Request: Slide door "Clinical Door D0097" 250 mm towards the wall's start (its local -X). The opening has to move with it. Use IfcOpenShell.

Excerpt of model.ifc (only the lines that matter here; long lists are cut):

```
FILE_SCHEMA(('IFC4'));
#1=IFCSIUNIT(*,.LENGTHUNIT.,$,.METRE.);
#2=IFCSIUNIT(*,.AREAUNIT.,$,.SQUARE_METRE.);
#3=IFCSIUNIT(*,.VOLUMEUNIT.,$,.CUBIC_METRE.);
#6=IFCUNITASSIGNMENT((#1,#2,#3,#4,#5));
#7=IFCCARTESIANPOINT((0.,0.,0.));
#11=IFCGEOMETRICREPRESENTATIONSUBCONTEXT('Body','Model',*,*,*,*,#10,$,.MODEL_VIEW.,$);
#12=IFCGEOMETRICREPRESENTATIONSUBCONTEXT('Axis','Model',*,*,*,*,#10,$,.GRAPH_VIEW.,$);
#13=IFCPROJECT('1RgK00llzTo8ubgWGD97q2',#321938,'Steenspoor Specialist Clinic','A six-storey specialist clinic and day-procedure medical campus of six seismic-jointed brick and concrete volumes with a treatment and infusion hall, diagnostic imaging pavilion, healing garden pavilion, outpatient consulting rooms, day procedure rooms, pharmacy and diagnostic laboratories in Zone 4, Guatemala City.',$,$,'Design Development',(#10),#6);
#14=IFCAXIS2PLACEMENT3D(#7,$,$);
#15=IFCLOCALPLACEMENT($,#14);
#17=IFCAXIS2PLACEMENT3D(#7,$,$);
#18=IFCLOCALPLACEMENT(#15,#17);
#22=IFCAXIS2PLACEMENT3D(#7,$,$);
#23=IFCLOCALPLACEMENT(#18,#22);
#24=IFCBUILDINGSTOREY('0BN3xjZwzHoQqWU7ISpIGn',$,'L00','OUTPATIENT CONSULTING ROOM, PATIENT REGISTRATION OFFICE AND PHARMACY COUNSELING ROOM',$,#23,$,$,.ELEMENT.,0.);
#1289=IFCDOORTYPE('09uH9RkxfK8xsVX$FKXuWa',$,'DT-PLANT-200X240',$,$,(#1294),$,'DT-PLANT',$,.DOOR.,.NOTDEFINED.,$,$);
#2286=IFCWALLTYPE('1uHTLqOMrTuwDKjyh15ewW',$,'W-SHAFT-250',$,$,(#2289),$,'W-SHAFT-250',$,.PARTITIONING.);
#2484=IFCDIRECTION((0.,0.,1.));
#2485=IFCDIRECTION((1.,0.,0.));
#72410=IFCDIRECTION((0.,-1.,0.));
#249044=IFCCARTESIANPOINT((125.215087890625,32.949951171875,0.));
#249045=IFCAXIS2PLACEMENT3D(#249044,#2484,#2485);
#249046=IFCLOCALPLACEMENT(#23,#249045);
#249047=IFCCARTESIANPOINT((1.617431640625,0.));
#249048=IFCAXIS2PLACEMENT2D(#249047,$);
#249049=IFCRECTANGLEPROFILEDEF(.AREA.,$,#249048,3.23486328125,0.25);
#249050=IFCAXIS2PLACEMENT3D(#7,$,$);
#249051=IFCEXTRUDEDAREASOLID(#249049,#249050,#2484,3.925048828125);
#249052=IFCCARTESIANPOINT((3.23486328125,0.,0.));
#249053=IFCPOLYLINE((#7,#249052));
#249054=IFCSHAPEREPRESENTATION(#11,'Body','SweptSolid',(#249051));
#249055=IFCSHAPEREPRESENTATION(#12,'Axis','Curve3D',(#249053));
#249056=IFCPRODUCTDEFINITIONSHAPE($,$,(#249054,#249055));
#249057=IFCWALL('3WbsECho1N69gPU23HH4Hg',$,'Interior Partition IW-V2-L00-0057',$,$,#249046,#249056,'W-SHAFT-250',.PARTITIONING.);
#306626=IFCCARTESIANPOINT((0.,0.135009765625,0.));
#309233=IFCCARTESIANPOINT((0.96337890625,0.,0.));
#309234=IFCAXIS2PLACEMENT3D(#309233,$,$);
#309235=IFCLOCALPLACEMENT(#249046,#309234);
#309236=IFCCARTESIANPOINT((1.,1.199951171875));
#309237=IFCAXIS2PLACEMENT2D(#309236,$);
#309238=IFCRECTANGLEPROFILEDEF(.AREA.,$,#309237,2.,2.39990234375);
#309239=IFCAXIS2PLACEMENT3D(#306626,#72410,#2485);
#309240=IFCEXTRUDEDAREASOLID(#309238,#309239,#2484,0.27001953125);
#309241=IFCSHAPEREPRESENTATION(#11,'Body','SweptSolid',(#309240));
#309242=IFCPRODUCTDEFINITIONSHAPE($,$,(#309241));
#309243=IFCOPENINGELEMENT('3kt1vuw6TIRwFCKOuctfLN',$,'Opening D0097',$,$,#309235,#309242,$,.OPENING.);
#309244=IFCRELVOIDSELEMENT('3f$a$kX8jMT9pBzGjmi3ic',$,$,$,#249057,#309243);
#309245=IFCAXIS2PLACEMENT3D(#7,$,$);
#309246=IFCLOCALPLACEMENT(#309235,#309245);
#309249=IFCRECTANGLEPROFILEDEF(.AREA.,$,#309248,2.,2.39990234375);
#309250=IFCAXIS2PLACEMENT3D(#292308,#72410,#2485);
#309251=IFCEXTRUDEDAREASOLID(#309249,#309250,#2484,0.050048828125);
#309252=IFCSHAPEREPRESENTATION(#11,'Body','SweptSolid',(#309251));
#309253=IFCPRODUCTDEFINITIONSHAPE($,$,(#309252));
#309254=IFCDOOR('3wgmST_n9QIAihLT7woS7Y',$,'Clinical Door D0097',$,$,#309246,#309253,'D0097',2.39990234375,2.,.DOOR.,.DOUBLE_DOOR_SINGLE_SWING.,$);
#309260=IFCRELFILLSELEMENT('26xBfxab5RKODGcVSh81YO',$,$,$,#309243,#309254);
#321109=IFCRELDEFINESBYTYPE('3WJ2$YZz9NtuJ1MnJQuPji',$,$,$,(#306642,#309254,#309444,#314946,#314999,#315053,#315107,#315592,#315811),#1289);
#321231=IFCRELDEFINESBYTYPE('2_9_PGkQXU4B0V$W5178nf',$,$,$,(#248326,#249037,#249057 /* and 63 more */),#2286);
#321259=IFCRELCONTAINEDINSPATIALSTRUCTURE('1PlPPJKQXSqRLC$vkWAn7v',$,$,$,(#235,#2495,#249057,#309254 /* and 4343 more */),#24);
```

```python
import ifcopenshell
import ifcopenshell.api.geometry
import ifcopenshell.util.placement
import ifcopenshell.util.unit

model = ifcopenshell.open("model.ifc")
unit_scale = ifcopenshell.util.unit.calculate_unit_scale(model)

door = model.by_guid("3wgmST_n9QIAihLT7woS7Y")
opening = door.FillsVoids[0].RelatingOpeningElement
wall = opening.VoidsElements[0].RelatingBuildingElement

wall_matrix = ifcopenshell.util.placement.get_local_placement(wall.ObjectPlacement)
shift = wall_matrix[:3, 0] * -0.25 / unit_scale
before = ifcopenshell.util.placement.get_local_placement(door.ObjectPlacement)[:3, 3].copy()

# The door is placed relative to its opening, so it follows when the opening moves.
matrix = ifcopenshell.util.placement.get_local_placement(opening.ObjectPlacement)
matrix[:3, 3] += shift
ifcopenshell.api.geometry.edit_object_placement(
    model, product=opening, matrix=matrix, is_si=False, should_transform_children=True
)

after = ifcopenshell.util.placement.get_local_placement(door.ObjectPlacement)[:3, 3]
print("door moved by", (after - before).round(3) + 0.0)

model.write("model_edited.ifc")
```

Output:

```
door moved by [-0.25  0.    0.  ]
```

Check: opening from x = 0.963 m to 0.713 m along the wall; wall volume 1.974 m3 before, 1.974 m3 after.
